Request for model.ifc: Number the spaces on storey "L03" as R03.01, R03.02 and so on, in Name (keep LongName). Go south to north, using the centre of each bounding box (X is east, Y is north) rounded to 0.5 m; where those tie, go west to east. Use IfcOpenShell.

First a look at what the model holds.

```python
import ifcopenshell
import ifcopenshell.util.element
import ifcopenshell.util.placement

model = ifcopenshell.open("model.ifc")
print(model.schema)
storey = next(s for s in model.by_type("IfcBuildingStorey") if s.Name == "L03")
spaces = [e for e in ifcopenshell.util.element.get_decomposition(storey) if e.is_a("IfcSpace")]
for e in sorted(spaces, key=lambda e: e.id()):
    origin = ifcopenshell.util.placement.get_local_placement(e.ObjectPlacement)[:3, 3]
    print(e.id(), e.Name, e.LongName, origin.round(2) + 0.0, sep=" | ")
```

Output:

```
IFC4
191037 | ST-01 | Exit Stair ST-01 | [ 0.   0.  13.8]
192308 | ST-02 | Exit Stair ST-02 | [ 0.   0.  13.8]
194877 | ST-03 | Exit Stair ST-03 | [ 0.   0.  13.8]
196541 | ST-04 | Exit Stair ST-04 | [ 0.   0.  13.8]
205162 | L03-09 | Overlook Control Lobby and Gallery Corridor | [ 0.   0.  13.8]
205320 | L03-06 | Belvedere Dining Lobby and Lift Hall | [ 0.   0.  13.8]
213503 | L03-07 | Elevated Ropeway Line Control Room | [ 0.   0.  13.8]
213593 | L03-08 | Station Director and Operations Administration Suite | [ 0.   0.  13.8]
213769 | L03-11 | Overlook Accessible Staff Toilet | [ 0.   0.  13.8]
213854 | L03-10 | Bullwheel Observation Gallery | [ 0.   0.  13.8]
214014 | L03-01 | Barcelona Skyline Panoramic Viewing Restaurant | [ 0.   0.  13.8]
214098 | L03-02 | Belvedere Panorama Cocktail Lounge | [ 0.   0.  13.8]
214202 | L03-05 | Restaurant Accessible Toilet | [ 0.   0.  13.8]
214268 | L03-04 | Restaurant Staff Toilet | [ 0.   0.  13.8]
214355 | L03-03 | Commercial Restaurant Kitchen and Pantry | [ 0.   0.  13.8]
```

```python
import ifcopenshell
import ifcopenshell.geom
import ifcopenshell.util.element
import ifcopenshell.util.shape

model = ifcopenshell.open("model.ifc")
settings = ifcopenshell.geom.settings()
settings.set("use-world-coords", True)


def centre(element):
    shape = ifcopenshell.geom.create_shape(settings, element)
    return ifcopenshell.util.shape.get_bbox_centroid(shape.geometry)


storey = next(s for s in model.by_type("IfcBuildingStorey") if s.Name == "L03")
spaces = [e for e in ifcopenshell.util.element.get_decomposition(storey) if e.is_a("IfcSpace")]

# Insertion points can sit at a corner or the storey origin, so sort by the geometry (in metres).
centres = {e: centre(e) for e in spaces}
spaces.sort(key=lambda e: (round(centres[e][1] / 0.5), centres[e][0]))

for i, e in enumerate(spaces, start=1):
    number = f"R03.{i:02d}"
    e.Name = number
    print(e.id(), number)

model.write("model-out.ifc")
```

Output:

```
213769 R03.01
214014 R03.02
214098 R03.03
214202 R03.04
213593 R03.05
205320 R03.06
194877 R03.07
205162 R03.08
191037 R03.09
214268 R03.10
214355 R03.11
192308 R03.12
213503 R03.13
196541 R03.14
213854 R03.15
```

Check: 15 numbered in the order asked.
